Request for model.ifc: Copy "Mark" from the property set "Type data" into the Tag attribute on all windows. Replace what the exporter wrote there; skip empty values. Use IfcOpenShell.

First a look at what the model holds.

```python
import ifcopenshell
import ifcopenshell.util.element

model = ifcopenshell.open("model.ifc")
print(model.schema)
windows = model.by_type("IfcWindow")
print(len(windows), "windows")
for e in windows[:8]:
    source = ifcopenshell.util.element.get_pset(e, "Type data", "Mark")
    target = e.Tag
    print(e.id(), repr(source), repr(target), sep=" | ")
```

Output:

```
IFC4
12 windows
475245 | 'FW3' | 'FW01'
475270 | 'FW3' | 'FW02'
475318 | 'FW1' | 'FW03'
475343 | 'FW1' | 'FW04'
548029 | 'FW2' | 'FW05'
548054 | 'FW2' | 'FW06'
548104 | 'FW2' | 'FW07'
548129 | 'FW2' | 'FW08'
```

```python
import ifcopenshell
import ifcopenshell.util.element

model = ifcopenshell.open("model.ifc")

count = 0
for e in model.by_type("IfcWindow"):
    value = ifcopenshell.util.element.get_pset(e, "Type data", "Mark")
    current = e.Tag
    if not value or not value.strip() or current == value:
        continue
    e.Tag = value
    count += 1

print(count, "windows updated")

model.write("model_updated.ifc")
```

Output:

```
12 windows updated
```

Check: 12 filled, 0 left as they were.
